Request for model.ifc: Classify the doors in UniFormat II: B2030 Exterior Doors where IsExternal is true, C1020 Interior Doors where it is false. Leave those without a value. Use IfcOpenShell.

First a look at what the model holds.

```python
import ifcopenshell
import ifcopenshell.util.element

model = ifcopenshell.open("model.ifc")
print(model.schema)
print("classifications:", [c.Name for c in model.by_type("IfcClassification")])
values = [ifcopenshell.util.element.get_pset(e, "Pset_DoorCommon", "IsExternal") for e in model.by_type("IfcDoor")]
for value in (True, False, None):
    print("IsExternal", value, values.count(value))
```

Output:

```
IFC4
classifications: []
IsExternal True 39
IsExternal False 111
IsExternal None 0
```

```python
import ifcopenshell
import ifcopenshell.api.classification
import ifcopenshell.util.element

model = ifcopenshell.open("model.ifc")

system = ifcopenshell.api.classification.add_classification(model, classification="UniFormat II")

doors = model.by_type("IfcDoor")
external = {e: ifcopenshell.util.element.get_pset(e, "Pset_DoorCommon", "IsExternal") for e in doors}
for flag, code, name in ((True, "B2030", "Exterior Doors"), (False, "C1020", "Interior Doors")):
    products = [e for e in doors if external[e] is flag]
    ifcopenshell.api.classification.add_reference(
        model, products=products, classification=system, identification=code, name=name
    )
    print(code, len(products))

model.write("model_updated.ifc")
```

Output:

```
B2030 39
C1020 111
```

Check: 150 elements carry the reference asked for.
